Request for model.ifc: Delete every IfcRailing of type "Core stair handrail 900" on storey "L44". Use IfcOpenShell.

First a look at what the model holds.

```python
import ifcopenshell
import ifcopenshell.util.element

model = ifcopenshell.open("model.ifc")
print(model.schema)
storey = next(s for s in model.by_type("IfcBuildingStorey") if s.Name == "L44")
railings = [e for e in ifcopenshell.util.element.get_decomposition(storey) if e.is_a("IfcRailing")]
seen = {}
for e in railings:
    element_type = ifcopenshell.util.element.get_type(e)
    name = element_type.Name if element_type not in (None, e) else None
    seen[name] = seen.get(name, 0) + 1
for name, count in sorted(seen.items(), key=str):
    print(count, "x", name)
```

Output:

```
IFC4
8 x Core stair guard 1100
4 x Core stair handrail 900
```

```python
import ifcopenshell
import ifcopenshell.api.root
import ifcopenshell.util.element

model = ifcopenshell.open("model.ifc")

storey = next(s for s in model.by_type("IfcBuildingStorey") if s.Name == "L44")
railings = [e for e in ifcopenshell.util.element.get_decomposition(storey) if e.is_a("IfcRailing")]
targets = [e for e in railings if (t := ifcopenshell.util.element.get_type(e)) not in (None, e) and t.Name == "Core stair handrail 900"]

for e in targets:
    ifcopenshell.api.root.remove_product(model, product=e)
print(len(targets), "removed")

model.write("model-out.ifc")
```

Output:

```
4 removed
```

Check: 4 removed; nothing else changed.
